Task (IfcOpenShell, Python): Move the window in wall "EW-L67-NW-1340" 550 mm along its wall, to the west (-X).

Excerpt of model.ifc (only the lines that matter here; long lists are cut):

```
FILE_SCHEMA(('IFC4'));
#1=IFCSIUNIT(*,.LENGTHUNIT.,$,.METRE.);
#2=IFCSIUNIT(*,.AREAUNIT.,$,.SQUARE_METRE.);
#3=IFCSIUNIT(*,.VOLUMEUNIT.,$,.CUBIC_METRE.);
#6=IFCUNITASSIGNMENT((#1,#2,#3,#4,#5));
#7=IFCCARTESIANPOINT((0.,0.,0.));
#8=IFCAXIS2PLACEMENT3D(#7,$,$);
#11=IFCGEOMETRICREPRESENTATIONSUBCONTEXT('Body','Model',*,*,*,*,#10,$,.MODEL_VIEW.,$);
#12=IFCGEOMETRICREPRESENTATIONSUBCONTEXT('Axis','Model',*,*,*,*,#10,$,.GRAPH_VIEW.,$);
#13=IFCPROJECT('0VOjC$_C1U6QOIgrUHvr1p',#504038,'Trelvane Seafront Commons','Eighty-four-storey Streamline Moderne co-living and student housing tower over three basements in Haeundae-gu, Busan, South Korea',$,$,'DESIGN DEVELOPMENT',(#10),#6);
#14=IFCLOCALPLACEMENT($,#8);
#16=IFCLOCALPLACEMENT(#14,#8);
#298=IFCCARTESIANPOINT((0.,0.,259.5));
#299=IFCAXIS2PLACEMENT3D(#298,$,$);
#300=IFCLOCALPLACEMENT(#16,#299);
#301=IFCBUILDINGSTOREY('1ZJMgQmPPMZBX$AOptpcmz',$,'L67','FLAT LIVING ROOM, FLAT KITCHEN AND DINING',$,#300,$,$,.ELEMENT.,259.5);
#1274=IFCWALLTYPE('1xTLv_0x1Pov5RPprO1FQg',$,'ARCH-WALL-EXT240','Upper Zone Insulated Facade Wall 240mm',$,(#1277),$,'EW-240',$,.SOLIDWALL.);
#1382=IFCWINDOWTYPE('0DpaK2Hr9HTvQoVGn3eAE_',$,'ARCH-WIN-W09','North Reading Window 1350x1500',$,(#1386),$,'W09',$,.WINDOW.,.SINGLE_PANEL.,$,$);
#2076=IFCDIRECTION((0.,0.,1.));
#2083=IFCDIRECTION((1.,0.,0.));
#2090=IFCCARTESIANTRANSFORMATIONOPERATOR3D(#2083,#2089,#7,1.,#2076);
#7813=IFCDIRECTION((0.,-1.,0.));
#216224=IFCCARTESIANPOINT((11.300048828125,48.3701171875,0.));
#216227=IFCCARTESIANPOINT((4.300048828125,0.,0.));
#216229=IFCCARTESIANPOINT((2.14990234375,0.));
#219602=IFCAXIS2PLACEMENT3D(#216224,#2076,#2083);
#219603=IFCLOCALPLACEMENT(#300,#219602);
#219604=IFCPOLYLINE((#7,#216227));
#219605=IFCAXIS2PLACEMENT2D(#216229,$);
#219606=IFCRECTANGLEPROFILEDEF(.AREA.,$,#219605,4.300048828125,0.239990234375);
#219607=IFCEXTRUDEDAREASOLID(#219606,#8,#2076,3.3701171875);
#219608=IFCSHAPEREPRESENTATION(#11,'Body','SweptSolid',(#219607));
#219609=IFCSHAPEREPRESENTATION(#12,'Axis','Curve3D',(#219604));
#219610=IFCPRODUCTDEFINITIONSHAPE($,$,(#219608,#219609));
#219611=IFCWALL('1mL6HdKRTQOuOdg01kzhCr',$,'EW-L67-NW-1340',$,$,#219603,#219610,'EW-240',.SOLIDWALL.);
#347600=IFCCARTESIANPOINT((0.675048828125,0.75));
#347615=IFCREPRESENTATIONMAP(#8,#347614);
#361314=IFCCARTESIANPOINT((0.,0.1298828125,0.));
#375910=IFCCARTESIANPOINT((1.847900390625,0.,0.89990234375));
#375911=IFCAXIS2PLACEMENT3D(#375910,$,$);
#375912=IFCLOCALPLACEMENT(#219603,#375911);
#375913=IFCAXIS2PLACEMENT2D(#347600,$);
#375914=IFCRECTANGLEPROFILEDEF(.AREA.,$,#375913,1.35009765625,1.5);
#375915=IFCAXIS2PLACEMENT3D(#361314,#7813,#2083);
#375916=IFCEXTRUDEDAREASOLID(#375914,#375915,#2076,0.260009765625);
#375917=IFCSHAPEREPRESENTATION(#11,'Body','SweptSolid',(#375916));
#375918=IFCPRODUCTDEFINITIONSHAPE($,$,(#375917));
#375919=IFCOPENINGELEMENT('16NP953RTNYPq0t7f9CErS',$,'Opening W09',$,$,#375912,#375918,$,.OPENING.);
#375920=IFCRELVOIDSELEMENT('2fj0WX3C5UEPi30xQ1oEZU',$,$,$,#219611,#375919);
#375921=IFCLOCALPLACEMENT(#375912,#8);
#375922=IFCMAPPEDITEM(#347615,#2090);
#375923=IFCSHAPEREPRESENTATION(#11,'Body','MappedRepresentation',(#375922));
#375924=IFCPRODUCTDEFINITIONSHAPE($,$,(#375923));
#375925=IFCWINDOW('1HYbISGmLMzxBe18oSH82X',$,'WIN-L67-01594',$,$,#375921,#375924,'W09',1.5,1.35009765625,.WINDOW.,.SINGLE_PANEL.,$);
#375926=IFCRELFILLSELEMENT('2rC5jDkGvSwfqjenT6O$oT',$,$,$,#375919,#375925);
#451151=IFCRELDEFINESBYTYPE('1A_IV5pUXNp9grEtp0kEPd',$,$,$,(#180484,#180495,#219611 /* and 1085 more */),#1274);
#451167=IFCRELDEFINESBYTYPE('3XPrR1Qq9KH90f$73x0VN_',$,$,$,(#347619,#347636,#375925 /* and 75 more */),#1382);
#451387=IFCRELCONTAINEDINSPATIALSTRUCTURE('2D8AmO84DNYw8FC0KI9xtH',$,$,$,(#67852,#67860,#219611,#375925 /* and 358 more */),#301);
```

```python
import ifcopenshell
import ifcopenshell.api.geometry
import ifcopenshell.util.placement
import ifcopenshell.util.unit

model = ifcopenshell.open("model.ifc")
unit_scale = ifcopenshell.util.unit.calculate_unit_scale(model)

window = model.by_guid("1HYbISGmLMzxBe18oSH82X")
opening = window.FillsVoids[0].RelatingOpeningElement
wall = opening.VoidsElements[0].RelatingBuildingElement

wall_matrix = ifcopenshell.util.placement.get_local_placement(wall.ObjectPlacement)
shift = wall_matrix[:3, 0] * -0.55 / unit_scale
before = ifcopenshell.util.placement.get_local_placement(window.ObjectPlacement)[:3, 3].copy()

# The window is placed relative to its opening, so it follows when the opening moves.
matrix = ifcopenshell.util.placement.get_local_placement(opening.ObjectPlacement)
matrix[:3, 3] += shift
ifcopenshell.api.geometry.edit_object_placement(
    model, product=opening, matrix=matrix, is_si=False, should_transform_children=True
)

after = ifcopenshell.util.placement.get_local_placement(window.ObjectPlacement)[:3, 3]
print("window moved by", (after - before).round(3) + 0.0)

model.write("model_updated.ifc")
```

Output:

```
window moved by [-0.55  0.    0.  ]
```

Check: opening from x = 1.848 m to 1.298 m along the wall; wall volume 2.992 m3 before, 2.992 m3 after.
